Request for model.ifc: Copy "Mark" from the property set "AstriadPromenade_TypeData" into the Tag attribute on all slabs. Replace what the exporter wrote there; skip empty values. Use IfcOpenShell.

First a look at what the model holds.

```python
import ifcopenshell
import ifcopenshell.util.element

model = ifcopenshell.open("model.ifc")
print(model.schema)
slabs = model.by_type("IfcSlab")
print(len(slabs), "slabs")
for e in slabs[:8]:
    source = ifcopenshell.util.element.get_pset(e, "AstriadPromenade_TypeData", "Mark")
    target = e.Tag
    print(e.id(), repr(source), repr(target), sep=" | ")
```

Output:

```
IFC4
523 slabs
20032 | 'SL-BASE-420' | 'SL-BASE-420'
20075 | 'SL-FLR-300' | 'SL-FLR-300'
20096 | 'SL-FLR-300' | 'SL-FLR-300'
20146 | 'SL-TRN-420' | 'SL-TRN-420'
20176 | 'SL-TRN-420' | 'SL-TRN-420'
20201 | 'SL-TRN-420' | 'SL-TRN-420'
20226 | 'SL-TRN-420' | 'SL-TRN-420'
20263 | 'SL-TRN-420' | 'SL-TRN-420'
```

```python
import ifcopenshell
import ifcopenshell.util.element

model = ifcopenshell.open("model.ifc")

count = 0
for e in model.by_type("IfcSlab"):
    value = ifcopenshell.util.element.get_pset(e, "AstriadPromenade_TypeData", "Mark")
    current = e.Tag
    if not value or not value.strip() or current == value:
        continue
    e.Tag = value
    count += 1

print(count, "slabs updated")

model.write("model_v2.ifc")
```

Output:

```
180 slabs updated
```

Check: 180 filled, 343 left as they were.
